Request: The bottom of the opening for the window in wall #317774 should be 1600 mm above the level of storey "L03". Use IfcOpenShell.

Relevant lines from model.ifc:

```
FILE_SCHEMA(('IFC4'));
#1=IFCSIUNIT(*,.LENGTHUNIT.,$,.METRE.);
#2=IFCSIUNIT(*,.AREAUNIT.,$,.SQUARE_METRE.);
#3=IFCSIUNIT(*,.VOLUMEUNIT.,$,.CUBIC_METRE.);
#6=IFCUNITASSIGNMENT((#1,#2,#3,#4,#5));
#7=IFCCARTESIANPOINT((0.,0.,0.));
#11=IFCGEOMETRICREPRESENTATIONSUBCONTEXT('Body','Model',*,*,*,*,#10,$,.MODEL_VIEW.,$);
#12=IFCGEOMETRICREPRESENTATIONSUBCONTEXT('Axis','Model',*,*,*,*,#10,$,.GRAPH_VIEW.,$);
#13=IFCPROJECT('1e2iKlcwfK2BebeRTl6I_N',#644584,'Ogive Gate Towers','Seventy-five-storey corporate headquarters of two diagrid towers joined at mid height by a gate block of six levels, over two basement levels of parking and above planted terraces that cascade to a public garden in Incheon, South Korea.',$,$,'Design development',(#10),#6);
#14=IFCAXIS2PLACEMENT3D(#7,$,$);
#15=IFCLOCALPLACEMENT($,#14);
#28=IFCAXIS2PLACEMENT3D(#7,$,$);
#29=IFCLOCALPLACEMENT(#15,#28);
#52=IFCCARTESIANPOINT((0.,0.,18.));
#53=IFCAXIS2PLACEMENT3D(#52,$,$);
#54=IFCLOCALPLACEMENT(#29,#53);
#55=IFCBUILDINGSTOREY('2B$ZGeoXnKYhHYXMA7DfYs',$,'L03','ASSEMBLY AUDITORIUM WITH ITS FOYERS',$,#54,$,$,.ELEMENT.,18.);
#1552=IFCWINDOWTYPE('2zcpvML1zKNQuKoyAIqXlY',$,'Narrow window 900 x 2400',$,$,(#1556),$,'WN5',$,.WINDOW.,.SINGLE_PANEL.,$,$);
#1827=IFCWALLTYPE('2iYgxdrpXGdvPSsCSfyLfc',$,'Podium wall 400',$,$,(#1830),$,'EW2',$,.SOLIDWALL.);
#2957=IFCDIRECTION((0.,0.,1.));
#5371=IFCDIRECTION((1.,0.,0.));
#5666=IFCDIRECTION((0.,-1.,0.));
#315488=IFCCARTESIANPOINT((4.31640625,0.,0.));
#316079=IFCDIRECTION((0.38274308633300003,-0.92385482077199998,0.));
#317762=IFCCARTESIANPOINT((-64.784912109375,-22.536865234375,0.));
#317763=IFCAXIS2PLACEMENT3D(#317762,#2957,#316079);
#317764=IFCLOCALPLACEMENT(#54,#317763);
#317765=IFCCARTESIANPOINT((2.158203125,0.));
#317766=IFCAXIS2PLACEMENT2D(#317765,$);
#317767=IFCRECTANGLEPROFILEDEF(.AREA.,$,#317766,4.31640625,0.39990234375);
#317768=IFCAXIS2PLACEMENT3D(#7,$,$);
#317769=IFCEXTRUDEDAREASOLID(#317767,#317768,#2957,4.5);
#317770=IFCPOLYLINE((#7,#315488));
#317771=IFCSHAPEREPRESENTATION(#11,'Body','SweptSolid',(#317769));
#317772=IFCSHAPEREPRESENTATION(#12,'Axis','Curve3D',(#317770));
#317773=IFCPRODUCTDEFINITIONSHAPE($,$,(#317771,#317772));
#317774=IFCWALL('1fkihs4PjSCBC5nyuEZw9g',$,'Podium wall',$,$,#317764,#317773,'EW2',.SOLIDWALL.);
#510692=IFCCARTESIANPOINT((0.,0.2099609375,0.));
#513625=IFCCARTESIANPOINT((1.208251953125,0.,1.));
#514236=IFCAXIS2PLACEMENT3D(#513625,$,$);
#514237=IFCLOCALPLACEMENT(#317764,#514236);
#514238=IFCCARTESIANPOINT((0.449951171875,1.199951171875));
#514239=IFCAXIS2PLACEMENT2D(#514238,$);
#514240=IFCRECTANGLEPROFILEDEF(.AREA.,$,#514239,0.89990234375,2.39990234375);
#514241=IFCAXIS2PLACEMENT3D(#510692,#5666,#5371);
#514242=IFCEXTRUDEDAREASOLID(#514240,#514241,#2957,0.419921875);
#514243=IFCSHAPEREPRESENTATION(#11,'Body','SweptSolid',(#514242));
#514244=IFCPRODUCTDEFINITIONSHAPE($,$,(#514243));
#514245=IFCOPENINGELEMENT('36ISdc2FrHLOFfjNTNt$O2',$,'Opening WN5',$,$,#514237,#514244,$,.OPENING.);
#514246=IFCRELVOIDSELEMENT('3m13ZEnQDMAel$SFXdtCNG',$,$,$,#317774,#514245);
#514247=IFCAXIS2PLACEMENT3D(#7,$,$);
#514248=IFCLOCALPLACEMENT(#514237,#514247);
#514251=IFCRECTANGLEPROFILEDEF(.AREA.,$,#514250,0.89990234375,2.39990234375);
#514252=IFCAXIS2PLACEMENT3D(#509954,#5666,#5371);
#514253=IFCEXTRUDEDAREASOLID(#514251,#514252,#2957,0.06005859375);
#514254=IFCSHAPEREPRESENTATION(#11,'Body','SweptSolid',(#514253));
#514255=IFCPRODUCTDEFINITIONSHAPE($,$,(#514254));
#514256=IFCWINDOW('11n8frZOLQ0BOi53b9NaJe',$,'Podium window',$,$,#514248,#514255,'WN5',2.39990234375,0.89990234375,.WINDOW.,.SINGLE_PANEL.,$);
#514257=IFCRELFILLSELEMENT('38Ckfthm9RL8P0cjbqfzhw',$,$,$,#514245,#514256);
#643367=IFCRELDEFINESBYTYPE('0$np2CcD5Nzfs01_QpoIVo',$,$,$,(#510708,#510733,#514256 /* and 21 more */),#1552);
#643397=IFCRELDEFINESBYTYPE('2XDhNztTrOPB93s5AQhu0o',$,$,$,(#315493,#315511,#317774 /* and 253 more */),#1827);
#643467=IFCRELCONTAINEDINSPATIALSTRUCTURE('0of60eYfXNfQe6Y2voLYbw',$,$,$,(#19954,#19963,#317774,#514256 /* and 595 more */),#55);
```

```python
import numpy as np
import ifcopenshell
import ifcopenshell.api.geometry
import ifcopenshell.geom
import ifcopenshell.util.element
import ifcopenshell.util.placement
import ifcopenshell.util.shape
import ifcopenshell.util.unit

model = ifcopenshell.open("model.ifc")
unit_scale = ifcopenshell.util.unit.calculate_unit_scale(model)

window = model.by_guid("11n8frZOLQ0BOi53b9NaJe")
opening = window.FillsVoids[0].RelatingOpeningElement
storey = ifcopenshell.util.element.get_container(window, ifc_class="IfcBuildingStorey")
level = ifcopenshell.util.placement.get_local_placement(storey.ObjectPlacement)[2, 3]

# The opening's origin need not be at the sill, so measure its lowest point.
shape = ifcopenshell.geom.create_shape(ifcopenshell.geom.settings(), opening)
bottom = ifcopenshell.util.shape.get_shape_bottom_elevation(shape, shape.geometry) / unit_scale
dz = level + 1.6 / unit_scale - bottom

shift = np.array([0.0, 0.0, dz])
# The window is placed relative to its opening, so it follows when the opening moves.
matrix = ifcopenshell.util.placement.get_local_placement(opening.ObjectPlacement)
matrix[:3, 3] += shift
ifcopenshell.api.geometry.edit_object_placement(
    model, product=opening, matrix=matrix, is_si=False, should_transform_children=True
)

print(f"moved by {dz * unit_scale:+.3f} m")

model.write("model-out.ifc")
```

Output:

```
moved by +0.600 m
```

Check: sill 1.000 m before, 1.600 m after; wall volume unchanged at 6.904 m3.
